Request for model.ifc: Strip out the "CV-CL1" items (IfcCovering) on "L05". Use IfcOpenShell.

First a look at what the model holds.

```python
import ifcopenshell
import ifcopenshell.util.element

model = ifcopenshell.open("model.ifc")
print(model.schema)
storey = next(s for s in model.by_type("IfcBuildingStorey") if s.Name == "L05")
coverings = [e for e in ifcopenshell.util.element.get_decomposition(storey) if e.is_a("IfcCovering")]
seen = {}
for e in coverings:
    element_type = ifcopenshell.util.element.get_type(e)
    name = element_type.Name if element_type not in (None, e) else None
    seen[name] = seen.get(name, 0) + 1
for name, count in sorted(seen.items(), key=str):
    print(count, "x", name)
```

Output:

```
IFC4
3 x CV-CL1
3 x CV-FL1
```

```python
import ifcopenshell
import ifcopenshell.api.root
import ifcopenshell.util.element

model = ifcopenshell.open("model.ifc")

storey = next(s for s in model.by_type("IfcBuildingStorey") if s.Name == "L05")
coverings = [e for e in ifcopenshell.util.element.get_decomposition(storey) if e.is_a("IfcCovering")]
targets = [e for e in coverings if (t := ifcopenshell.util.element.get_type(e)) not in (None, e) and t.Name == "CV-CL1"]

for e in targets:
    ifcopenshell.api.root.remove_product(model, product=e)
print(len(targets), "removed")

model.write("model_v2.ifc")
```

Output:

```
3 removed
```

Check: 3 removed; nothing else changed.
